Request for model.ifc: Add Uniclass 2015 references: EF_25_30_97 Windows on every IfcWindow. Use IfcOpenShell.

First a look at what the model holds.

```python
import ifcopenshell

model = ifcopenshell.open("model.ifc")
print(model.schema)
print("classifications:", [c.Name for c in model.by_type("IfcClassification")])
for ifc_class in ("IfcDoor", "IfcRoof", "IfcStair", "IfcWall", "IfcWindow"):
    print(ifc_class, len(model.by_type(ifc_class)))
```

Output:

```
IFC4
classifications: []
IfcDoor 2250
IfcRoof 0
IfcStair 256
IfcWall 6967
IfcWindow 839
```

```python
import ifcopenshell
import ifcopenshell.api.classification

model = ifcopenshell.open("model.ifc")

system = ifcopenshell.api.classification.add_classification(model, classification="Uniclass 2015")

codes = {
    "IfcWindow": ("EF_25_30_97", "Windows"),
}
for ifc_class, (code, name) in codes.items():
    products = model.by_type(ifc_class)
    ifcopenshell.api.classification.add_reference(
        model, products=products, classification=system, identification=code, name=name
    )
    print(code, len(products))

model.write("model_edited.ifc")
```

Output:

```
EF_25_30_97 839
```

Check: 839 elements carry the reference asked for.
